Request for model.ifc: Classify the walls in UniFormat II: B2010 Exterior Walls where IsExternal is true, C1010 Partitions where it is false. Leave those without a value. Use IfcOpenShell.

First a look at what the model holds.

```python
import ifcopenshell
import ifcopenshell.util.element

model = ifcopenshell.open("model.ifc")
print(model.schema)
print("classifications:", [c.Name for c in model.by_type("IfcClassification")])
values = [ifcopenshell.util.element.get_pset(e, "Pset_WallCommon", "IsExternal") for e in model.by_type("IfcWall")]
for value in (True, False, None):
    print("IsExternal", value, values.count(value))
```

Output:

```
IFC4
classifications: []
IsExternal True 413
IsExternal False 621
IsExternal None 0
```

```python
import ifcopenshell
import ifcopenshell.api.classification
import ifcopenshell.util.element

model = ifcopenshell.open("model.ifc")

system = ifcopenshell.api.classification.add_classification(model, classification="UniFormat II")

walls = model.by_type("IfcWall")
external = {e: ifcopenshell.util.element.get_pset(e, "Pset_WallCommon", "IsExternal") for e in walls}
for flag, code, name in ((True, "B2010", "Exterior Walls"), (False, "C1010", "Partitions")):
    products = [e for e in walls if external[e] is flag]
    ifcopenshell.api.classification.add_reference(
        model, products=products, classification=system, identification=code, name=name
    )
    print(code, len(products))

model.write("model_v2.ifc")
```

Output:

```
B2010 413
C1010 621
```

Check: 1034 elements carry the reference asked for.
